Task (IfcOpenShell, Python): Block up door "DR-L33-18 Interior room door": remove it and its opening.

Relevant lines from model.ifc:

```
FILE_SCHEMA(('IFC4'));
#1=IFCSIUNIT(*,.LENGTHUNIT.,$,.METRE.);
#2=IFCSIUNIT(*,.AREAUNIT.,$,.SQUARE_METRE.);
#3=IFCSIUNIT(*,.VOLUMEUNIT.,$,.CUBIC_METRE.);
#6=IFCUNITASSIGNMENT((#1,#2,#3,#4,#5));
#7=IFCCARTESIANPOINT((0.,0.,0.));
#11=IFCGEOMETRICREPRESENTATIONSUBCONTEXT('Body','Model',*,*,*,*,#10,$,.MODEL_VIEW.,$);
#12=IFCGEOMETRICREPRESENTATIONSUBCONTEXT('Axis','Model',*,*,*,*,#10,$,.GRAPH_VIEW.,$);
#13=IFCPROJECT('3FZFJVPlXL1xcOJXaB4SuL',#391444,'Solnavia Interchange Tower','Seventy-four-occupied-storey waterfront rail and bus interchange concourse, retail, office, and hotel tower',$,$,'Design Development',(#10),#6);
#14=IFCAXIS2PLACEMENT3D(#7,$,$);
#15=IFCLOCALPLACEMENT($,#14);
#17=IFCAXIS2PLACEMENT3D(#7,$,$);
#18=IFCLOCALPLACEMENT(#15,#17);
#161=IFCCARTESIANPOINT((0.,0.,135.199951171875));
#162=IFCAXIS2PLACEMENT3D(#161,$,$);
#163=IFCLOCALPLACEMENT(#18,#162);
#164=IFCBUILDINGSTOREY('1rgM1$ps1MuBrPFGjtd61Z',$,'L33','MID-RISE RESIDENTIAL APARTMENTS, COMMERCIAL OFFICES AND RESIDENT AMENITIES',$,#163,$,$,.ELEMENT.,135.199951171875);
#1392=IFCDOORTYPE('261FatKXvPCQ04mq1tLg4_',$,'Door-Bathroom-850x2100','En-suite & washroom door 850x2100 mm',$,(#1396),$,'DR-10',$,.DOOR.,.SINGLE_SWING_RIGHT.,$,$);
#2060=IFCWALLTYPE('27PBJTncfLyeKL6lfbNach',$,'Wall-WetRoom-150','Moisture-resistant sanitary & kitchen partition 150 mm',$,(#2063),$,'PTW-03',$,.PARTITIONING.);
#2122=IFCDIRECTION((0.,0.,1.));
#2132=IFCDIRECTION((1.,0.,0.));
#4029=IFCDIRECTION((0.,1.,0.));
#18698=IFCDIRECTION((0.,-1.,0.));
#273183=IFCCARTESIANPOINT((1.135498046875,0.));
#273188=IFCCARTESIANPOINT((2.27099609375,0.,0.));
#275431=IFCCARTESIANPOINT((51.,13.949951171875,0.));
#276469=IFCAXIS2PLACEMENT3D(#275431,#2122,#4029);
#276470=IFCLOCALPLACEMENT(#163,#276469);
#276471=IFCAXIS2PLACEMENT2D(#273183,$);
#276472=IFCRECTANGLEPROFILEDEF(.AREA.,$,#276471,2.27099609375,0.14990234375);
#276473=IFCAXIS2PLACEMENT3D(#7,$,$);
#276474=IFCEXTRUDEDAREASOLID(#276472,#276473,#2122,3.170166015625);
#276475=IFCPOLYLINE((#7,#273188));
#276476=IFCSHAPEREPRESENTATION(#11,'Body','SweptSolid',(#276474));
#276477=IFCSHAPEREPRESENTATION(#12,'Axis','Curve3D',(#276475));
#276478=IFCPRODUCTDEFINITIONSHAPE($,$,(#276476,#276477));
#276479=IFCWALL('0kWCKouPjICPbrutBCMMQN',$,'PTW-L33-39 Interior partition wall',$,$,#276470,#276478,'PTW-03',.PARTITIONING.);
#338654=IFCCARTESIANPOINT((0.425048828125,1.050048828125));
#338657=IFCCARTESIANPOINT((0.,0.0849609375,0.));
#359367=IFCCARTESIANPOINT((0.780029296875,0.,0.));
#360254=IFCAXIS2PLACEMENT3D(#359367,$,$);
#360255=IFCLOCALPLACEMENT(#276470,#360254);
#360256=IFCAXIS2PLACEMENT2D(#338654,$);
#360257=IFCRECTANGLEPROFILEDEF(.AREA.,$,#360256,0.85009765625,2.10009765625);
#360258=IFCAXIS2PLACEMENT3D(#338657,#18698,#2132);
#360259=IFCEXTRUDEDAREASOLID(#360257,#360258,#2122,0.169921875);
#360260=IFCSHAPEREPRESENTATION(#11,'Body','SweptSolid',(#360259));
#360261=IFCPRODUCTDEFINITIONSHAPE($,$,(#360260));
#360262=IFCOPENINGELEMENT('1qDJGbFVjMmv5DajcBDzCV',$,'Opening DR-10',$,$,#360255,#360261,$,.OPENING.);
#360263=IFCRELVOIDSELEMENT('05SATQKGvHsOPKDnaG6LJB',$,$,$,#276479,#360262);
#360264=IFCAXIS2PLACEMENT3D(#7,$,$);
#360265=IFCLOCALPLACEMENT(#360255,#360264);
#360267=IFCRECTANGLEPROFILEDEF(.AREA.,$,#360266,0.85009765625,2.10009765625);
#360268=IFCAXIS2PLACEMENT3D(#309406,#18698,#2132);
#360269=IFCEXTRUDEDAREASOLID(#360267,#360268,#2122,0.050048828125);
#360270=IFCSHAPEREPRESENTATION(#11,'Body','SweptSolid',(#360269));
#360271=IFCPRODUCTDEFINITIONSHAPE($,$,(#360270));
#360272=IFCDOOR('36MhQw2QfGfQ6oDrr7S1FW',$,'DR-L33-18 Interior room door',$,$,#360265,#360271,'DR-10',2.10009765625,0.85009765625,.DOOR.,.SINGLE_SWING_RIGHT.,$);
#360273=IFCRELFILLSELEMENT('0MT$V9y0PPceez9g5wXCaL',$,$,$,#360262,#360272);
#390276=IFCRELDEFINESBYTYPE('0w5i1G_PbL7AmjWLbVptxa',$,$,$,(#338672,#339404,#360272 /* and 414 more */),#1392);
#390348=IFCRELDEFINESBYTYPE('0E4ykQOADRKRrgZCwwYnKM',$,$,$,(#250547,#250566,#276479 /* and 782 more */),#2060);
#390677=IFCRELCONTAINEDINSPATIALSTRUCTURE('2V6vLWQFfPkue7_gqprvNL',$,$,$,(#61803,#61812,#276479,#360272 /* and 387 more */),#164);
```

```python
import ifcopenshell
import ifcopenshell.api.feature
import ifcopenshell.api.root
import ifcopenshell.geom
import ifcopenshell.util.shape

model = ifcopenshell.open("model.ifc")
settings = ifcopenshell.geom.settings()


def volume(element):
    """Net volume in cubic metres, openings subtracted."""
    shape = ifcopenshell.geom.create_shape(settings, element)
    return ifcopenshell.util.shape.get_volume(shape.geometry)


door = model.by_guid("36MhQw2QfGfQ6oDrr7S1FW")
opening = door.FillsVoids[0].RelatingOpeningElement
wall = opening.VoidsElements[0].RelatingBuildingElement
before = volume(wall)

ifcopenshell.api.root.remove_product(model, product=door)
ifcopenshell.api.feature.remove_feature(model, feature=opening)

after = volume(wall)

print(f"wall volume {before:.3f} -> {after:.3f} m3")

model.write("model_v2.ifc")
```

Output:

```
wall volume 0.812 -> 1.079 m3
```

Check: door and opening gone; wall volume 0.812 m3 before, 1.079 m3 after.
